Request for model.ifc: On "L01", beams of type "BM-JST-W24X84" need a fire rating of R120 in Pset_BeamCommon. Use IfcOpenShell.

First a look at what the model holds.

```python
import ifcopenshell
import ifcopenshell.util.element

model = ifcopenshell.open("model.ifc")
print(model.schema)
storey = next(s for s in model.by_type("IfcBuildingStorey") if s.Name == "L01")
beams = [e for e in ifcopenshell.util.element.get_decomposition(storey) if e.is_a("IfcBeam")]
seen = {}
for e in beams:
    element_type = ifcopenshell.util.element.get_type(e)
    key = (element_type.Name if element_type != e and element_type else None, ifcopenshell.util.element.get_pset(e, "Pset_BeamCommon", "FireRating"))
    seen[key] = seen.get(key, 0) + 1
for (name, value), count in sorted(seen.items(), key=str):
    print(count, "x", name, "|", value)
```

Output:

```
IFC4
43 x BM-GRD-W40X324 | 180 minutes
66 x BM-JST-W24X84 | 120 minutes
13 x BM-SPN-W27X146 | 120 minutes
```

```python
import ifcopenshell
import ifcopenshell.api.pset
import ifcopenshell.util.element

model = ifcopenshell.open("model.ifc")

storey = next(s for s in model.by_type("IfcBuildingStorey") if s.Name == "L01")
beams = [e for e in ifcopenshell.util.element.get_decomposition(storey) if e.is_a("IfcBeam")]

count = 0
for e in beams:
    element_type = ifcopenshell.util.element.get_type(e)
    if element_type in (None, e) or element_type.Name != "BM-JST-W24X84":
        continue
    found = ifcopenshell.util.element.get_pset(e, "Pset_BeamCommon", should_inherit=False)
    if found:
        pset = model.by_id(found["id"])
        if len(ifcopenshell.util.element.get_elements_by_pset(pset)) > 1:
            pset = ifcopenshell.api.pset.unshare_pset(model, products=[e], pset=pset)[0]
    else:
        pset = ifcopenshell.api.pset.add_pset(model, product=e, name="Pset_BeamCommon")
    ifcopenshell.api.pset.edit_pset(model, pset=pset, properties={"FireRating": "R120"})
    count += 1

print(count, "beams updated")

model.write("model_rev.ifc")
```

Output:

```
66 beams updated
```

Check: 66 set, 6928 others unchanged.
